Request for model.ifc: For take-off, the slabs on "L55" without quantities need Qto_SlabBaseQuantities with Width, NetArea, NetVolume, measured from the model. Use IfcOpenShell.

First a look at what the model holds.

```python
import ifcopenshell
import ifcopenshell.util.element
import ifcopenshell.util.unit

model = ifcopenshell.open("model.ifc")
print(model.schema)
for unit_type in ("LENGTHUNIT", "AREAUNIT", "VOLUMEUNIT"):
    print(unit_type, ifcopenshell.util.unit.calculate_unit_scale(model, unit_type))
storey = next(s for s in model.by_type("IfcBuildingStorey") if s.Name == "L55")
slabs = [e for e in ifcopenshell.util.element.get_decomposition(storey) if e.is_a("IfcSlab")]
for e in sorted(slabs, key=lambda e: e.id()):
    print(e.id(), e.is_a(), e.Name, list(ifcopenshell.util.element.get_psets(e, qtos_only=True)), sep=" | ")
```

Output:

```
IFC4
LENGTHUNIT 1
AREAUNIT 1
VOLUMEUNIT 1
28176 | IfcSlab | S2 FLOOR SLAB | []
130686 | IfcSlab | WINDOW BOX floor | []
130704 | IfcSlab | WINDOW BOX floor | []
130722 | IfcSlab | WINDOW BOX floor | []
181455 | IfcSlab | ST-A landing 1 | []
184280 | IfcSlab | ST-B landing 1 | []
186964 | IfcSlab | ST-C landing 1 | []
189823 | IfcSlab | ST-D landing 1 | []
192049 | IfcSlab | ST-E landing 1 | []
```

```python
import ifcopenshell
import ifcopenshell.api.pset
import ifcopenshell.geom
import ifcopenshell.util.element
import ifcopenshell.util.shape
import ifcopenshell.util.unit

model = ifcopenshell.open("model.ifc")
unit_scale = ifcopenshell.util.unit.calculate_unit_scale(model)
area_scale = ifcopenshell.util.unit.calculate_unit_scale(model, "AREAUNIT")
volume_scale = ifcopenshell.util.unit.calculate_unit_scale(model, "VOLUMEUNIT")
settings = ifcopenshell.geom.settings()

storey = next(s for s in model.by_type("IfcBuildingStorey") if s.Name == "L55")
slabs = [e for e in ifcopenshell.util.element.get_decomposition(storey) if e.is_a("IfcSlab")]

for e in sorted(slabs, key=lambda e: e.id()):
    if ifcopenshell.util.element.get_psets(e, qtos_only=True, should_inherit=False):
        continue
    # Geometry comes back in metres, in the element's own axes.
    shape = ifcopenshell.geom.create_shape(settings, e)
    values = {
        "Width": ifcopenshell.util.shape.get_z(shape.geometry) / unit_scale,
        "NetArea": ifcopenshell.util.shape.get_footprint_area(shape.geometry) / area_scale,
        "NetVolume": ifcopenshell.util.shape.get_volume(shape.geometry) / volume_scale,
    }
    qto = ifcopenshell.api.pset.add_qto(model, product=e, name="Qto_SlabBaseQuantities")
    ifcopenshell.api.pset.edit_qto(model, qto=qto, properties=values)
    print(e.id(), {k: round(v, 3) for k, v in values.items()})

model.write("model_edited.ifc")
```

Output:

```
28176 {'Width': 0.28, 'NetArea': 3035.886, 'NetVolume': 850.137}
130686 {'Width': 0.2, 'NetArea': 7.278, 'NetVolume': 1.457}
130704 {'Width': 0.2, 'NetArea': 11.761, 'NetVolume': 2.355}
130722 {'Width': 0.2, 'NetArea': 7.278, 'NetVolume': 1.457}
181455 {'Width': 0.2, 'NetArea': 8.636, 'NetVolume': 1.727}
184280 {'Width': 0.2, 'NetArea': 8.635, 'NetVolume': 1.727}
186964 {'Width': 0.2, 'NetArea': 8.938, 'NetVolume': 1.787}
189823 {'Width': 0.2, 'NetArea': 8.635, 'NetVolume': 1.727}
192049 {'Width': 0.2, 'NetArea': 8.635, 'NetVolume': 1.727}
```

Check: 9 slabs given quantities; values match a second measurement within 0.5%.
